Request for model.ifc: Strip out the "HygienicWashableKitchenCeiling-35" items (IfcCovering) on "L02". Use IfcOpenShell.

First a look at what the model holds.

```python
import ifcopenshell
import ifcopenshell.util.element

model = ifcopenshell.open("model.ifc")
print(model.schema)
storey = next(s for s in model.by_type("IfcBuildingStorey") if s.Name == "L02")
coverings = [e for e in ifcopenshell.util.element.get_decomposition(storey) if e.is_a("IfcCovering")]
seen = {}
for e in coverings:
    element_type = ifcopenshell.util.element.get_type(e)
    name = element_type.Name if element_type not in (None, e) else None
    seen[name] = seen.get(name, 0) + 1
for name, count in sorted(seen.items(), key=str):
    print(count, "x", name)
```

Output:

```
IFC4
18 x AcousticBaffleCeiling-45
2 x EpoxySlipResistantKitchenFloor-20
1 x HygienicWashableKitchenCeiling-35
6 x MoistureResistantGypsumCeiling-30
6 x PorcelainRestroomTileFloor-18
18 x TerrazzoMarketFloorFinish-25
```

```python
import ifcopenshell
import ifcopenshell.api.root
import ifcopenshell.util.element

model = ifcopenshell.open("model.ifc")

storey = next(s for s in model.by_type("IfcBuildingStorey") if s.Name == "L02")
coverings = [e for e in ifcopenshell.util.element.get_decomposition(storey) if e.is_a("IfcCovering")]
targets = [e for e in coverings if (t := ifcopenshell.util.element.get_type(e)) not in (None, e) and t.Name == "HygienicWashableKitchenCeiling-35"]

for e in targets:
    ifcopenshell.api.root.remove_product(model, product=e)
print(len(targets), "removed")

model.write("model-out.ifc")
```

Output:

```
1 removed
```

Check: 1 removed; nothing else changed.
